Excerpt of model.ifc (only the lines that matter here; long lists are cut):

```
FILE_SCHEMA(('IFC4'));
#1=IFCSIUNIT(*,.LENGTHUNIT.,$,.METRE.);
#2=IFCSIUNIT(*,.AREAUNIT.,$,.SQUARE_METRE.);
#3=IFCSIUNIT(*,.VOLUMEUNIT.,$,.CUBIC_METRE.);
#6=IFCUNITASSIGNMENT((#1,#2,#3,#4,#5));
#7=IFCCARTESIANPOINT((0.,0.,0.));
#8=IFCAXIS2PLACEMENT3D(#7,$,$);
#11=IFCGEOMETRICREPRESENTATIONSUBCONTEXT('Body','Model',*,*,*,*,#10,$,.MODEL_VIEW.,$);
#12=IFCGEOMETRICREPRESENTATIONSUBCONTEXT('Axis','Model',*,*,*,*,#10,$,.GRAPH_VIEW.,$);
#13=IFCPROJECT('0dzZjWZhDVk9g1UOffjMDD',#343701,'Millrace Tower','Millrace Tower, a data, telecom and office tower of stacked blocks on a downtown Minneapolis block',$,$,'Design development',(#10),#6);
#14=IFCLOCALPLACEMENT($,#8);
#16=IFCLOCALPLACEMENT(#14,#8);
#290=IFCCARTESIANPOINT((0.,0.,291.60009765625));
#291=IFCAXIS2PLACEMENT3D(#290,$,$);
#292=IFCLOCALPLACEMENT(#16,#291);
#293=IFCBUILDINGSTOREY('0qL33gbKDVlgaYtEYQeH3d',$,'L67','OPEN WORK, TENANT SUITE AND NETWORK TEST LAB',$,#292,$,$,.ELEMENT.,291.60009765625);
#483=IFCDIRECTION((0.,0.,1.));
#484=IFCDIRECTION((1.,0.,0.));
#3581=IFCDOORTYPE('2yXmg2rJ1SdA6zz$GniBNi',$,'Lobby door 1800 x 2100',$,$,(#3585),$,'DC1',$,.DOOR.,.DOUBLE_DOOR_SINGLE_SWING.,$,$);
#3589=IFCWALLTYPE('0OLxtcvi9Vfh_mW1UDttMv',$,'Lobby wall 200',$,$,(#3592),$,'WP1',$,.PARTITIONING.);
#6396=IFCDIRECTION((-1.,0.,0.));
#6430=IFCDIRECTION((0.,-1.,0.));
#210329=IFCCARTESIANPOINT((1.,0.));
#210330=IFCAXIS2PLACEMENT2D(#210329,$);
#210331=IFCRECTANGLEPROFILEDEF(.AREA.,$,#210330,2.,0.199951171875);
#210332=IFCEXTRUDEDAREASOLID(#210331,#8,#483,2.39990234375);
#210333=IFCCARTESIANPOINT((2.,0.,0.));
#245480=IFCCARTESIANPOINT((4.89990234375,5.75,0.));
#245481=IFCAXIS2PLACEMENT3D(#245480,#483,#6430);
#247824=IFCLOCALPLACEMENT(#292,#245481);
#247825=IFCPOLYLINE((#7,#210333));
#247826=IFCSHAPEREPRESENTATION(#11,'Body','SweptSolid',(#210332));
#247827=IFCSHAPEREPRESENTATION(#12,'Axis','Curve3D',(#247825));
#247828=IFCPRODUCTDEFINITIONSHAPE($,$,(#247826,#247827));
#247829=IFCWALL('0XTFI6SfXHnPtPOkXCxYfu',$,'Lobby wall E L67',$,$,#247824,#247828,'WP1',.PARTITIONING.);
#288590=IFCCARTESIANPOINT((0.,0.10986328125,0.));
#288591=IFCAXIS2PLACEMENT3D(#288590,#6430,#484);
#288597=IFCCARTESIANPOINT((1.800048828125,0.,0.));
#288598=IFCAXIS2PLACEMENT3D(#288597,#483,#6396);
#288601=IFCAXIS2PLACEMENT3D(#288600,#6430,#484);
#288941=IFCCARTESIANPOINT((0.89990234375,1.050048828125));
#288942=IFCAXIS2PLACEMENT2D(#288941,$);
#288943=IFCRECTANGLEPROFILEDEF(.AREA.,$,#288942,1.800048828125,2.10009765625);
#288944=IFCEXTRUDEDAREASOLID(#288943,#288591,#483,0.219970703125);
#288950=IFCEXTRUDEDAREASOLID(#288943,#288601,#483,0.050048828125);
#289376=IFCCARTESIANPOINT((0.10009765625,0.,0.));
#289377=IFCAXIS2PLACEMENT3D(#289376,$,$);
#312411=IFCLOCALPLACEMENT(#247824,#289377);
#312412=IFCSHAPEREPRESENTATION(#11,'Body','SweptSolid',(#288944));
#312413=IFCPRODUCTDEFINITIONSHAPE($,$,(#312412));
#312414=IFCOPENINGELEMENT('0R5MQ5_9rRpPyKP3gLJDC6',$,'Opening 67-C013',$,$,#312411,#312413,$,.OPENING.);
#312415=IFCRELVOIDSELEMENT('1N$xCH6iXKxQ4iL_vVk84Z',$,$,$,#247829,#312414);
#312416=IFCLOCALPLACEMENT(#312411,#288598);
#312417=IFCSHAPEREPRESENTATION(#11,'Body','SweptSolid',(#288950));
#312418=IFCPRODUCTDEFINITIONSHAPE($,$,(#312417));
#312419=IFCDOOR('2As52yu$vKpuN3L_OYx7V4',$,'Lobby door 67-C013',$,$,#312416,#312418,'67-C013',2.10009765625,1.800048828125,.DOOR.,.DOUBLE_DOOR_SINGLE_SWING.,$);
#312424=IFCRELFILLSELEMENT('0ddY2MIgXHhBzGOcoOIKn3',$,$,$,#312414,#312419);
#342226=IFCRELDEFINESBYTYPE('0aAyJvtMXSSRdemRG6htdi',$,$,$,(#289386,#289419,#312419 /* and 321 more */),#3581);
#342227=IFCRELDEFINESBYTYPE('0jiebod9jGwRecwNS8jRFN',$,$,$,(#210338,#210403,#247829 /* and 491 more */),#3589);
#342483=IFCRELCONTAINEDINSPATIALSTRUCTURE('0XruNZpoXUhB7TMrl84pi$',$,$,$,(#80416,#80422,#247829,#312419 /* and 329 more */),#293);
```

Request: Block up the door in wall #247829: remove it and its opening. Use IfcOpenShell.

```python
import ifcopenshell
import ifcopenshell.api.feature
import ifcopenshell.api.root
import ifcopenshell.geom
import ifcopenshell.util.shape

model = ifcopenshell.open("model.ifc")
settings = ifcopenshell.geom.settings()


def volume(element):
    """Net volume in cubic metres, openings subtracted."""
    shape = ifcopenshell.geom.create_shape(settings, element)
    return ifcopenshell.util.shape.get_volume(shape.geometry)


door = model.by_id(312419)
opening = door.FillsVoids[0].RelatingOpeningElement
wall = opening.VoidsElements[0].RelatingBuildingElement
before = volume(wall)

ifcopenshell.api.root.remove_product(model, product=door)
ifcopenshell.api.feature.remove_feature(model, feature=opening)

after = volume(wall)

print(f"wall volume {before:.3f} -> {after:.3f} m3")

model.write("model_updated.ifc")
```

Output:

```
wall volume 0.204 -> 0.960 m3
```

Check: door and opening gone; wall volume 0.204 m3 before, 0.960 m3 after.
